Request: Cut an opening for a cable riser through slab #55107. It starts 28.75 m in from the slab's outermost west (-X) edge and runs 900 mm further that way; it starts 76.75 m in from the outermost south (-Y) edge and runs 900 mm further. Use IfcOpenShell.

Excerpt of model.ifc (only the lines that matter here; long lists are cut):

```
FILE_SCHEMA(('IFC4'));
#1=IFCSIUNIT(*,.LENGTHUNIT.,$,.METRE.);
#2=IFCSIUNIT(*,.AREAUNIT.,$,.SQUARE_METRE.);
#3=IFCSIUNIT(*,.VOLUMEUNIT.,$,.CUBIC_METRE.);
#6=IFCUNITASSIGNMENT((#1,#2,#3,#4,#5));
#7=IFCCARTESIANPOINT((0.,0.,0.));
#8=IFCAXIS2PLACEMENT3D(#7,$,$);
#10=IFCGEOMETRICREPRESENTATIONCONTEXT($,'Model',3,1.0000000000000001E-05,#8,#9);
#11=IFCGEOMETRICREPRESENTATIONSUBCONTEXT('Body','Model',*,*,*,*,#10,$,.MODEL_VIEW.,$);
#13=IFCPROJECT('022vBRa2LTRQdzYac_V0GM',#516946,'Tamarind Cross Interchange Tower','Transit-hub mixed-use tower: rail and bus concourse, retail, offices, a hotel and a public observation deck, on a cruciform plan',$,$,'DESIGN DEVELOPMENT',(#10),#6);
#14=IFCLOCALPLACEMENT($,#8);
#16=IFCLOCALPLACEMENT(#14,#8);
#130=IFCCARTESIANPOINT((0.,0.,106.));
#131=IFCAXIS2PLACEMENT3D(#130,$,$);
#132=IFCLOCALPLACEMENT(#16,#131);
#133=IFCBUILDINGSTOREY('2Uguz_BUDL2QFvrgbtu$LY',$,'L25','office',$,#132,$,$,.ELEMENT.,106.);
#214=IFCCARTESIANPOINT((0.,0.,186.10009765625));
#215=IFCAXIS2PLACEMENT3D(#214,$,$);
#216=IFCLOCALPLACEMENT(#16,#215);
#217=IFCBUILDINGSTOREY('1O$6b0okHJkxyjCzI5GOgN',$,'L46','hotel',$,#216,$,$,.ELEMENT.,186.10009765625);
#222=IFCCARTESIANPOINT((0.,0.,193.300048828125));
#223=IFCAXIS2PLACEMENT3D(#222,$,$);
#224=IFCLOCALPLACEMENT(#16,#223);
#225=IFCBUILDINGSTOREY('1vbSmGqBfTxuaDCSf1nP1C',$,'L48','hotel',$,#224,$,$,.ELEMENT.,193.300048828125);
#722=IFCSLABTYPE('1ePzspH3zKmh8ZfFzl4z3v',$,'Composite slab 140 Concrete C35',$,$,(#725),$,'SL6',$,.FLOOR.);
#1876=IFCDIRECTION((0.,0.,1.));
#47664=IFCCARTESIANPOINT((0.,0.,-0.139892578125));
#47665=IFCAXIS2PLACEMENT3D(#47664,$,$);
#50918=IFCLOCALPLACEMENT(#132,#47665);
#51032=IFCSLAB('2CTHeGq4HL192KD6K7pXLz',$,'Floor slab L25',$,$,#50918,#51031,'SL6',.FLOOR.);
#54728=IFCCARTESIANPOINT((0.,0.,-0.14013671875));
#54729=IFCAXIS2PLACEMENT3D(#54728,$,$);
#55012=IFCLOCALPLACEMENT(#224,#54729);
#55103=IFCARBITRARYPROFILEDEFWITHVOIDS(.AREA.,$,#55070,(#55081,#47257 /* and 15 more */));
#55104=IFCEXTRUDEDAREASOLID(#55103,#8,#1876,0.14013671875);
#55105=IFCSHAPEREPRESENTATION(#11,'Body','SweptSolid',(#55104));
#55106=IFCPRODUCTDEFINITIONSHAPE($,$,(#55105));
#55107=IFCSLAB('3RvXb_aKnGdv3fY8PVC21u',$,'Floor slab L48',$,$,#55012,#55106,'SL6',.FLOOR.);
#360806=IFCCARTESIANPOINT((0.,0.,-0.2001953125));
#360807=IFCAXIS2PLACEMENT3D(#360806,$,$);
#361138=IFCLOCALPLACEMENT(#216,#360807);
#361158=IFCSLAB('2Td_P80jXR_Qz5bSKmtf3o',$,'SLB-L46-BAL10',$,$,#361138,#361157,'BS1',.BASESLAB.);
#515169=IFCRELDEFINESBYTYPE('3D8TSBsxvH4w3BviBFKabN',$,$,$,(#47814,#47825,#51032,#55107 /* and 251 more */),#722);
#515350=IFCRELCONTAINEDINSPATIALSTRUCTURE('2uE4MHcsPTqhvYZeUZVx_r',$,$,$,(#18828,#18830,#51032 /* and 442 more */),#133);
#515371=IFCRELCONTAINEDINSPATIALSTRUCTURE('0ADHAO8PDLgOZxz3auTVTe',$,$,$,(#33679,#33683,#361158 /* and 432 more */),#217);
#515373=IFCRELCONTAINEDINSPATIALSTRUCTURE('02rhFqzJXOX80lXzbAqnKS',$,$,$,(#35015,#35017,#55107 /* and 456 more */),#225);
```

```python
import numpy as np
import ifcopenshell
import ifcopenshell.api.feature
import ifcopenshell.api.geometry
import ifcopenshell.api.root
import ifcopenshell.geom
import ifcopenshell.util.placement
import ifcopenshell.util.representation
import ifcopenshell.util.shape
import ifcopenshell.util.unit

model = ifcopenshell.open("model.ifc")
unit_scale = ifcopenshell.util.unit.calculate_unit_scale(model)
settings = ifcopenshell.geom.settings()


def volume(element):
    """Net volume in cubic metres, openings subtracted."""
    shape = ifcopenshell.geom.create_shape(settings, element)
    return ifcopenshell.util.shape.get_volume(shape.geometry)


slab = model.by_guid("3RvXb_aKnGdv3fY8PVC21u")
before = volume(slab)

# Extent in the slab's own axes, in metres. The edges named are its -X and -Y sides.
slab_shape = ifcopenshell.geom.create_shape(settings, slab)
vertices = ifcopenshell.util.shape.get_vertices(slab_shape.geometry)
x_min, y_min, bottom = vertices.min(axis=0)
top = vertices[:, 2].max()

opening = ifcopenshell.api.root.create_entity(model, ifc_class="IfcOpeningElement", name="Cable riser opening", predefined_type="OPENING")
context = ifcopenshell.util.representation.get_context(model, "Model", "Body", "MODEL_VIEW")
width, depth = 0.9, 0.9
outline = [(0.0, 0.0), (width, 0.0), (width, depth), (0.0, depth), (0.0, 0.0)]
# Overshoot both faces by 50 mm so the cut is clean.
shape = ifcopenshell.api.geometry.add_slab_representation(
    model, context=context, depth=top - bottom + 0.1, polyline=outline
)
ifcopenshell.api.geometry.assign_representation(model, product=opening, representation=shape)

matrix = ifcopenshell.util.placement.get_local_placement(slab.ObjectPlacement)
matrix[:, 3] = matrix @ np.append(np.array([x_min + 28.75, y_min + 76.75, bottom - 0.05]) / unit_scale, 1.0)
ifcopenshell.api.geometry.edit_object_placement(model, product=opening, matrix=matrix, is_si=False)
ifcopenshell.api.feature.add_feature(model, feature=opening, element=slab)

after = volume(slab)

print(f"slab volume {before:.3f} -> {after:.3f} m3")

model.write("model_rev.ifc")
```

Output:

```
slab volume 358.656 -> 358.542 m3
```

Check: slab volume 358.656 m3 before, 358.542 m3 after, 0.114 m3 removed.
